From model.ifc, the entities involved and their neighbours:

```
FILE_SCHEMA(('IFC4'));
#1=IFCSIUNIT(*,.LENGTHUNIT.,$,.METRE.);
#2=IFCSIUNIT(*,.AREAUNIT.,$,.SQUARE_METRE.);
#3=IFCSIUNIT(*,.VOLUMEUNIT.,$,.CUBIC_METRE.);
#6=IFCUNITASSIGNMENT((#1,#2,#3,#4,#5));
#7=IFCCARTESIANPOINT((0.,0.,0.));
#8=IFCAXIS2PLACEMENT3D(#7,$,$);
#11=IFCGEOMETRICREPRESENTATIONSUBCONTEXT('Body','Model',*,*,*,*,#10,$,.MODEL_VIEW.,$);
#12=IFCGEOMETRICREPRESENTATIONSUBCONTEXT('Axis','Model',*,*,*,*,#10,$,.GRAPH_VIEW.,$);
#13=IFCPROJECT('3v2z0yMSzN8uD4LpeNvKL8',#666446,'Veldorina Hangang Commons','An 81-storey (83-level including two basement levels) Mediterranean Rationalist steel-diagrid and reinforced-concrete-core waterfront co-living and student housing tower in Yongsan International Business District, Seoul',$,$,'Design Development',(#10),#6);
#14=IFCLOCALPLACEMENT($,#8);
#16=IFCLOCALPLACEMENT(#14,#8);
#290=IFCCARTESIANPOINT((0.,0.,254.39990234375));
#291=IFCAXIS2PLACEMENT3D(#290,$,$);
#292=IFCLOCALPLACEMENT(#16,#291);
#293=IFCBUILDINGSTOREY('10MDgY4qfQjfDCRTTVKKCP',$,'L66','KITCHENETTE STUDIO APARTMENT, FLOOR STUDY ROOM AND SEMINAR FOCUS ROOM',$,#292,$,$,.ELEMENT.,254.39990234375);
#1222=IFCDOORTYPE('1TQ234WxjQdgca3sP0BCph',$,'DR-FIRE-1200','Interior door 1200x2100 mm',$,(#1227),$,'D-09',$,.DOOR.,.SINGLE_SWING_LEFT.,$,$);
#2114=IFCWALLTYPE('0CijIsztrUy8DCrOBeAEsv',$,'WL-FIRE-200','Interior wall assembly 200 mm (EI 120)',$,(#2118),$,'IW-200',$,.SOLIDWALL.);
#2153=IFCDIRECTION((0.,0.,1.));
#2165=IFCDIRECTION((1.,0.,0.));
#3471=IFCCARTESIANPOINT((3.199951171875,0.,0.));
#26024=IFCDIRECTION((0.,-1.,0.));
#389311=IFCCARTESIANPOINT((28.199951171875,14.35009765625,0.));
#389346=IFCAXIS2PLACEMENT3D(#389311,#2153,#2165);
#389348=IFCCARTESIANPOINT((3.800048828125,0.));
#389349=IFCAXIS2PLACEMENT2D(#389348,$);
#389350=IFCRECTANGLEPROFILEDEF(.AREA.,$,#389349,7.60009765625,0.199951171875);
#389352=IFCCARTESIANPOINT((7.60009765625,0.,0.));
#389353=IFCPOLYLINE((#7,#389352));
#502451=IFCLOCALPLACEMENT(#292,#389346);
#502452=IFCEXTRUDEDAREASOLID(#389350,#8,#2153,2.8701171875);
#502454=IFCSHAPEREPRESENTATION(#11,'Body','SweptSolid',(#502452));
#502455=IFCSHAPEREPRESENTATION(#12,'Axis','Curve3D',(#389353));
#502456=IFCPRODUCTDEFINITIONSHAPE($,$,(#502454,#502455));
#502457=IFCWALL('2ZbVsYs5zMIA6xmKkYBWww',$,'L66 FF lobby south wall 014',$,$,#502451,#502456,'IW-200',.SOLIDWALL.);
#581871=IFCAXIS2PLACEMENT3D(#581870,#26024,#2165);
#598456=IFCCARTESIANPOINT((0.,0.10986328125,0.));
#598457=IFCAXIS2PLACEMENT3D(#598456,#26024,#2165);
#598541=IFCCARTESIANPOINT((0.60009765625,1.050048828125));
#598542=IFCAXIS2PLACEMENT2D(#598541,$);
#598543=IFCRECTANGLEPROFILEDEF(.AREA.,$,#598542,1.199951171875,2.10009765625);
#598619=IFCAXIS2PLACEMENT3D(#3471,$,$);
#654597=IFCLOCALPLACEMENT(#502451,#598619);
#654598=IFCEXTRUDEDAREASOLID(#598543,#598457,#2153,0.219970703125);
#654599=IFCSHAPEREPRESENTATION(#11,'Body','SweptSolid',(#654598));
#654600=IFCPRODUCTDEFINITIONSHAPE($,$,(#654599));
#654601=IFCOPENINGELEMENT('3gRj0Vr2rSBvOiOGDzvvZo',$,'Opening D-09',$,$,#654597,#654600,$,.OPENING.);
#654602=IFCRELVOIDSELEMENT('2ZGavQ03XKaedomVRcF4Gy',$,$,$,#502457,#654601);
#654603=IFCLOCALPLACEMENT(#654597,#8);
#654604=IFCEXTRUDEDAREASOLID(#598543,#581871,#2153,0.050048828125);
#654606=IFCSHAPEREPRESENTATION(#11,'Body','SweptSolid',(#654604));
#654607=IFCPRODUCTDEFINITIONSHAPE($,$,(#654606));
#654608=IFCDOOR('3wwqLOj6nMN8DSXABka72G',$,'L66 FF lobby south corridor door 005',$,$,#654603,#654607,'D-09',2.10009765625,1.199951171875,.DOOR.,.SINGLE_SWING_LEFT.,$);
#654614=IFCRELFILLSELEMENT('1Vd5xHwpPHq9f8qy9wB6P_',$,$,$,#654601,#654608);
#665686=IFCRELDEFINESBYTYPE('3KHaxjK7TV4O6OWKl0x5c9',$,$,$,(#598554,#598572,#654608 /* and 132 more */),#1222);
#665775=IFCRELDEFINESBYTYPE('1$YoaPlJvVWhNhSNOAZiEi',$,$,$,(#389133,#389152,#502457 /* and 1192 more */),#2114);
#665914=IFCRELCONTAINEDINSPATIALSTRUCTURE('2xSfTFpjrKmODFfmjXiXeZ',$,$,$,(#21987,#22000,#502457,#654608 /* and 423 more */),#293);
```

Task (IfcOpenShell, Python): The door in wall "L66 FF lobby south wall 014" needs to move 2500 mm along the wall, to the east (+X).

```python
import ifcopenshell
import ifcopenshell.api.geometry
import ifcopenshell.util.placement

model = ifcopenshell.open("model.ifc")

door = model.by_id(654608)
opening = door.FillsVoids[0].RelatingOpeningElement
wall = opening.VoidsElements[0].RelatingBuildingElement

wall_matrix = ifcopenshell.util.placement.get_local_placement(wall.ObjectPlacement)
shift = wall_matrix[:3, 0] * 2.5
before = ifcopenshell.util.placement.get_local_placement(door.ObjectPlacement)[:3, 3].copy()

# The door is placed relative to its opening, so it follows when the opening moves.
matrix = ifcopenshell.util.placement.get_local_placement(opening.ObjectPlacement)
matrix[:3, 3] += shift
ifcopenshell.api.geometry.edit_object_placement(
    model, product=opening, matrix=matrix, is_si=False, should_transform_children=True
)

after = ifcopenshell.util.placement.get_local_placement(door.ObjectPlacement)[:3, 3]
print("door moved by", (after - before).round(3) + 0.0)

model.write("model_rev.ifc")
```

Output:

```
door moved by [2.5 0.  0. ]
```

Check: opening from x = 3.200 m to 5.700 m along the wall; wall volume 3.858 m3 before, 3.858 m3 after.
